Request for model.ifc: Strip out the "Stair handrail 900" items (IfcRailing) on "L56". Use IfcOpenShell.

First a look at what the model holds.

```python
import ifcopenshell
import ifcopenshell.util.element

model = ifcopenshell.open("model.ifc")
print(model.schema)
storey = next(s for s in model.by_type("IfcBuildingStorey") if s.Name == "L56")
railings = [e for e in ifcopenshell.util.element.get_decomposition(storey) if e.is_a("IfcRailing")]
seen = {}
for e in railings:
    element_type = ifcopenshell.util.element.get_type(e)
    name = element_type.Name if element_type not in (None, e) else None
    seen[name] = seen.get(name, 0) + 1
for name, count in sorted(seen.items(), key=str):
    print(count, "x", name)
```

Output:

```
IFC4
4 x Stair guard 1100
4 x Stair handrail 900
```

```python
import ifcopenshell
import ifcopenshell.api.root
import ifcopenshell.util.element

model = ifcopenshell.open("model.ifc")

storey = next(s for s in model.by_type("IfcBuildingStorey") if s.Name == "L56")
railings = [e for e in ifcopenshell.util.element.get_decomposition(storey) if e.is_a("IfcRailing")]
targets = [e for e in railings if (t := ifcopenshell.util.element.get_type(e)) not in (None, e) and t.Name == "Stair handrail 900"]

for e in targets:
    ifcopenshell.api.root.remove_product(model, product=e)
print(len(targets), "removed")

model.write("model_edited.ifc")
```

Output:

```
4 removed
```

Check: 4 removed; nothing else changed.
